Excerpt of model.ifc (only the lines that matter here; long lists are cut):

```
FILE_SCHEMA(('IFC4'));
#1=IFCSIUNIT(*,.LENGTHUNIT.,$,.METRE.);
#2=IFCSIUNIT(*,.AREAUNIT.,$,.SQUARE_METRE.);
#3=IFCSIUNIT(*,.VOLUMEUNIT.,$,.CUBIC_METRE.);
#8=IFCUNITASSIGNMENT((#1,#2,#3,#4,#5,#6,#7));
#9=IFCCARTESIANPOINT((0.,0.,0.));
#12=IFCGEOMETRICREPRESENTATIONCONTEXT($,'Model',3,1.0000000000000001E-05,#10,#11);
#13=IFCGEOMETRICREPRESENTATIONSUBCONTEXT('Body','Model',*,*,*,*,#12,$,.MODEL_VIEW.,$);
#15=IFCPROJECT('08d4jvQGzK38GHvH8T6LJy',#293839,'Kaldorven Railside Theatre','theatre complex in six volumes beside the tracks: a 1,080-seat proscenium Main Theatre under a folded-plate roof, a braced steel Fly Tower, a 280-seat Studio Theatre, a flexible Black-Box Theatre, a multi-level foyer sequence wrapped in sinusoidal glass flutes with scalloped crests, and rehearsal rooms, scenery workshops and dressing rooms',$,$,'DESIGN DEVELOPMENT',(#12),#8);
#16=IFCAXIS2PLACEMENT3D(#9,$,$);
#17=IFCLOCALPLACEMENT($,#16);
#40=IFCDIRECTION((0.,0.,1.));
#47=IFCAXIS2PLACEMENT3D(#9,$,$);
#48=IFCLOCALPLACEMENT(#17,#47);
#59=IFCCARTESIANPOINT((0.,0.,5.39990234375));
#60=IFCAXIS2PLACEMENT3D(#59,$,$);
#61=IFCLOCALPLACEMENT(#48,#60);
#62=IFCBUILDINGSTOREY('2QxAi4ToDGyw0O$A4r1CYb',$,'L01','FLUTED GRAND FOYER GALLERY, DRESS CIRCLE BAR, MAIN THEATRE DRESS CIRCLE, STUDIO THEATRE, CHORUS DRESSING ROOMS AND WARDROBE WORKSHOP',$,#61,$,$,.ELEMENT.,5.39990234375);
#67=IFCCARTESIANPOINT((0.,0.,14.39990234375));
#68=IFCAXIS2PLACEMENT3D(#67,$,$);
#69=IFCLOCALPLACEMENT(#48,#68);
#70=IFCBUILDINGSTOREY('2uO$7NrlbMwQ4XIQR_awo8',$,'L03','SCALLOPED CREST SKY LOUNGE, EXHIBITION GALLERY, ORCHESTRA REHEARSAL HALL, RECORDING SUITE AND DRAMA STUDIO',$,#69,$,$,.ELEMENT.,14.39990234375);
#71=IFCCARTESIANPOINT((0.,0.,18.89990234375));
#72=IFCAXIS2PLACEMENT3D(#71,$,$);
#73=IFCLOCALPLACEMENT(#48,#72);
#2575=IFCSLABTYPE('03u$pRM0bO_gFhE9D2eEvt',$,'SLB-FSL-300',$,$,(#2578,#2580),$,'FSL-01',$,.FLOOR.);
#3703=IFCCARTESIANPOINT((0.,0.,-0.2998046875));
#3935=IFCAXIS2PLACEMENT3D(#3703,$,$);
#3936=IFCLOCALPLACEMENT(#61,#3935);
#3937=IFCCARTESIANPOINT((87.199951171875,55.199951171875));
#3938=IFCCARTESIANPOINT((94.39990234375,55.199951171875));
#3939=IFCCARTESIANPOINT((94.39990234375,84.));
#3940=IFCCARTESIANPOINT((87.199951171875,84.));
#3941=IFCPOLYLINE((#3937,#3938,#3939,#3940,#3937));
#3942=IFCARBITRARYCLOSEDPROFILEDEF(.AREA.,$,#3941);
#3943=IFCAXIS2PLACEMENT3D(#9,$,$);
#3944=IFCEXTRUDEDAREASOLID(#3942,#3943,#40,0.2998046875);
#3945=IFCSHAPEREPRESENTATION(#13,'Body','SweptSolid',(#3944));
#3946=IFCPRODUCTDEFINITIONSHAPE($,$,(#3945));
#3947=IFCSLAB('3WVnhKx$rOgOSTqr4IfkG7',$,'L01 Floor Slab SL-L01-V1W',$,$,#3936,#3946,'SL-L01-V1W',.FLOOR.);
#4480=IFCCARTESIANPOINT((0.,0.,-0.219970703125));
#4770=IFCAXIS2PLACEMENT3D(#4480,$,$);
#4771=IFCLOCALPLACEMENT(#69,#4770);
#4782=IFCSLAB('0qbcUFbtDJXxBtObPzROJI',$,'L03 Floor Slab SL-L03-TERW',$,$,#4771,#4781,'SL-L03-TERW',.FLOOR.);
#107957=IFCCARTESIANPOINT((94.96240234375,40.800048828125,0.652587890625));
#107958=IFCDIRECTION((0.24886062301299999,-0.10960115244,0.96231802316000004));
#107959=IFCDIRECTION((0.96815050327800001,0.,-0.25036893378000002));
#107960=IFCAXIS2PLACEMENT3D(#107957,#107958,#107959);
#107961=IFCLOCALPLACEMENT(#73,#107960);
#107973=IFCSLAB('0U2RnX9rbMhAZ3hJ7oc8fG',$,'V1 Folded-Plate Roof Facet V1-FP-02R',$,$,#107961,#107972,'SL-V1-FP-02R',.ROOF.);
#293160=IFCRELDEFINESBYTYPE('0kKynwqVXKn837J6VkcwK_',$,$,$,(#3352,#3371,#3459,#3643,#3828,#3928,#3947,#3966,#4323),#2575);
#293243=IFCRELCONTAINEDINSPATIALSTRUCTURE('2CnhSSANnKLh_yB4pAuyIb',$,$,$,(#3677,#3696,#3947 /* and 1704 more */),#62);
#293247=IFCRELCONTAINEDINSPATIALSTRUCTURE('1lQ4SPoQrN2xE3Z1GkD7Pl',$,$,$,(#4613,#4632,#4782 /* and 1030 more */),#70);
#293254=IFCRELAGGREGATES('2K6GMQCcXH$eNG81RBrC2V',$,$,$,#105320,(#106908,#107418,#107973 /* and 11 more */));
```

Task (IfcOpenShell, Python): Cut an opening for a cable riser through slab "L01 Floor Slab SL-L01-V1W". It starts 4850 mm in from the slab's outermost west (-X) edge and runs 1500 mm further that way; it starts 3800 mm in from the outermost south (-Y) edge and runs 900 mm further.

```python
import numpy as np
import ifcopenshell
import ifcopenshell.api.feature
import ifcopenshell.api.geometry
import ifcopenshell.api.root
import ifcopenshell.geom
import ifcopenshell.util.placement
import ifcopenshell.util.representation
import ifcopenshell.util.shape
import ifcopenshell.util.unit

model = ifcopenshell.open("model.ifc")
unit_scale = ifcopenshell.util.unit.calculate_unit_scale(model)
settings = ifcopenshell.geom.settings()


def volume(element):
    """Net volume in cubic metres, openings subtracted."""
    shape = ifcopenshell.geom.create_shape(settings, element)
    return ifcopenshell.util.shape.get_volume(shape.geometry)


slab = model.by_guid("3WVnhKx$rOgOSTqr4IfkG7")
before = volume(slab)

# Extent in the slab's own axes, in metres. The edges named are its -X and -Y sides.
slab_shape = ifcopenshell.geom.create_shape(settings, slab)
vertices = ifcopenshell.util.shape.get_vertices(slab_shape.geometry)
x_min, y_min, bottom = vertices.min(axis=0)
top = vertices[:, 2].max()

opening = ifcopenshell.api.root.create_entity(model, ifc_class="IfcOpeningElement", name="Cable riser opening", predefined_type="OPENING")
context = ifcopenshell.util.representation.get_context(model, "Model", "Body", "MODEL_VIEW")
width, depth = 1.5, 0.9
outline = [(0.0, 0.0), (width, 0.0), (width, depth), (0.0, depth), (0.0, 0.0)]
# Overshoot both faces by 50 mm so the cut is clean.
shape = ifcopenshell.api.geometry.add_slab_representation(
    model, context=context, depth=top - bottom + 0.1, polyline=outline
)
ifcopenshell.api.geometry.assign_representation(model, product=opening, representation=shape)

matrix = ifcopenshell.util.placement.get_local_placement(slab.ObjectPlacement)
matrix[:, 3] = matrix @ np.append(np.array([x_min + 4.85, y_min + 3.8, bottom - 0.05]) / unit_scale, 1.0)
ifcopenshell.api.geometry.edit_object_placement(model, product=opening, matrix=matrix, is_si=False)
ifcopenshell.api.feature.add_feature(model, feature=opening, element=slab)

after = volume(slab)

print(f"slab volume {before:.3f} -> {after:.3f} m3")

model.write("model_updated.ifc")
```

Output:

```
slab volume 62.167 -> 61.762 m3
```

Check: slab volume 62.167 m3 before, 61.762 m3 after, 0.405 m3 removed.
